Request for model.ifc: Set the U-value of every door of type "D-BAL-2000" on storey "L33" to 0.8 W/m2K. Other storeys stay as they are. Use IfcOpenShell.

First a look at what the model holds.

```python
import ifcopenshell
import ifcopenshell.util.element

model = ifcopenshell.open("model.ifc")
print(model.schema)
storey = next(s for s in model.by_type("IfcBuildingStorey") if s.Name == "L33")
doors = [e for e in ifcopenshell.util.element.get_decomposition(storey) if e.is_a("IfcDoor")]
seen = {}
for e in doors:
    element_type = ifcopenshell.util.element.get_type(e)
    key = (element_type.Name if element_type != e and element_type else None, ifcopenshell.util.element.get_pset(e, "Pset_DoorCommon", "ThermalTransmittance"))
    seen[key] = seen.get(key, 0) + 1
for (name, value), count in sorted(seen.items(), key=str):
    print(count, "x", name, "|", value)
```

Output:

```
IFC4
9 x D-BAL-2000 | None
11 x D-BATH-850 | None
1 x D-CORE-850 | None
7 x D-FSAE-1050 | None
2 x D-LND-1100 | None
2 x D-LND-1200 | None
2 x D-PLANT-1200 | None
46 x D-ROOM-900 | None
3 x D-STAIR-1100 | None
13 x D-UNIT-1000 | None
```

```python
import ifcopenshell
import ifcopenshell.api.pset
import ifcopenshell.util.element

model = ifcopenshell.open("model.ifc")

storey = next(s for s in model.by_type("IfcBuildingStorey") if s.Name == "L33")
doors = [e for e in ifcopenshell.util.element.get_decomposition(storey) if e.is_a("IfcDoor")]

count = 0
for e in doors:
    element_type = ifcopenshell.util.element.get_type(e)
    if element_type in (None, e) or element_type.Name != "D-BAL-2000":
        continue
    # add_pset returns the element's existing set when there is one.
    pset = ifcopenshell.api.pset.add_pset(model, product=e, name="Pset_DoorCommon")
    ifcopenshell.api.pset.edit_pset(model, pset=pset, properties={"ThermalTransmittance": 0.8})
    count += 1

print(count, "doors updated")

model.write("model_updated.ifc")
```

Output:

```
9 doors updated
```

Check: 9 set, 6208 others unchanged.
